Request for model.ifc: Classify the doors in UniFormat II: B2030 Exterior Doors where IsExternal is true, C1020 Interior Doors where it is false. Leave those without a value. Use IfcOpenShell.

First a look at what the model holds.

```python
import ifcopenshell
import ifcopenshell.util.element

model = ifcopenshell.open("model.ifc")
print(model.schema)
print("classifications:", [c.Name for c in model.by_type("IfcClassification")])
values = [ifcopenshell.util.element.get_pset(e, "Pset_DoorCommon", "IsExternal") for e in model.by_type("IfcDoor")]
for value in (True, False, None):
    print("IsExternal", value, values.count(value))
```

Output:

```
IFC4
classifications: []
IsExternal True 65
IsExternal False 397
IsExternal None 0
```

```python
import ifcopenshell
import ifcopenshell.api.classification
import ifcopenshell.util.element

model = ifcopenshell.open("model.ifc")

system = ifcopenshell.api.classification.add_classification(model, classification="UniFormat II")

doors = model.by_type("IfcDoor")
external = {e: ifcopenshell.util.element.get_pset(e, "Pset_DoorCommon", "IsExternal") for e in doors}
for flag, code, name in ((True, "B2030", "Exterior Doors"), (False, "C1020", "Interior Doors")):
    products = [e for e in doors if external[e] is flag]
    ifcopenshell.api.classification.add_reference(
        model, products=products, classification=system, identification=code, name=name
    )
    print(code, len(products))

model.write("model_updated.ifc")
```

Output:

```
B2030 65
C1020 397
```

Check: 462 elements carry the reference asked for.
